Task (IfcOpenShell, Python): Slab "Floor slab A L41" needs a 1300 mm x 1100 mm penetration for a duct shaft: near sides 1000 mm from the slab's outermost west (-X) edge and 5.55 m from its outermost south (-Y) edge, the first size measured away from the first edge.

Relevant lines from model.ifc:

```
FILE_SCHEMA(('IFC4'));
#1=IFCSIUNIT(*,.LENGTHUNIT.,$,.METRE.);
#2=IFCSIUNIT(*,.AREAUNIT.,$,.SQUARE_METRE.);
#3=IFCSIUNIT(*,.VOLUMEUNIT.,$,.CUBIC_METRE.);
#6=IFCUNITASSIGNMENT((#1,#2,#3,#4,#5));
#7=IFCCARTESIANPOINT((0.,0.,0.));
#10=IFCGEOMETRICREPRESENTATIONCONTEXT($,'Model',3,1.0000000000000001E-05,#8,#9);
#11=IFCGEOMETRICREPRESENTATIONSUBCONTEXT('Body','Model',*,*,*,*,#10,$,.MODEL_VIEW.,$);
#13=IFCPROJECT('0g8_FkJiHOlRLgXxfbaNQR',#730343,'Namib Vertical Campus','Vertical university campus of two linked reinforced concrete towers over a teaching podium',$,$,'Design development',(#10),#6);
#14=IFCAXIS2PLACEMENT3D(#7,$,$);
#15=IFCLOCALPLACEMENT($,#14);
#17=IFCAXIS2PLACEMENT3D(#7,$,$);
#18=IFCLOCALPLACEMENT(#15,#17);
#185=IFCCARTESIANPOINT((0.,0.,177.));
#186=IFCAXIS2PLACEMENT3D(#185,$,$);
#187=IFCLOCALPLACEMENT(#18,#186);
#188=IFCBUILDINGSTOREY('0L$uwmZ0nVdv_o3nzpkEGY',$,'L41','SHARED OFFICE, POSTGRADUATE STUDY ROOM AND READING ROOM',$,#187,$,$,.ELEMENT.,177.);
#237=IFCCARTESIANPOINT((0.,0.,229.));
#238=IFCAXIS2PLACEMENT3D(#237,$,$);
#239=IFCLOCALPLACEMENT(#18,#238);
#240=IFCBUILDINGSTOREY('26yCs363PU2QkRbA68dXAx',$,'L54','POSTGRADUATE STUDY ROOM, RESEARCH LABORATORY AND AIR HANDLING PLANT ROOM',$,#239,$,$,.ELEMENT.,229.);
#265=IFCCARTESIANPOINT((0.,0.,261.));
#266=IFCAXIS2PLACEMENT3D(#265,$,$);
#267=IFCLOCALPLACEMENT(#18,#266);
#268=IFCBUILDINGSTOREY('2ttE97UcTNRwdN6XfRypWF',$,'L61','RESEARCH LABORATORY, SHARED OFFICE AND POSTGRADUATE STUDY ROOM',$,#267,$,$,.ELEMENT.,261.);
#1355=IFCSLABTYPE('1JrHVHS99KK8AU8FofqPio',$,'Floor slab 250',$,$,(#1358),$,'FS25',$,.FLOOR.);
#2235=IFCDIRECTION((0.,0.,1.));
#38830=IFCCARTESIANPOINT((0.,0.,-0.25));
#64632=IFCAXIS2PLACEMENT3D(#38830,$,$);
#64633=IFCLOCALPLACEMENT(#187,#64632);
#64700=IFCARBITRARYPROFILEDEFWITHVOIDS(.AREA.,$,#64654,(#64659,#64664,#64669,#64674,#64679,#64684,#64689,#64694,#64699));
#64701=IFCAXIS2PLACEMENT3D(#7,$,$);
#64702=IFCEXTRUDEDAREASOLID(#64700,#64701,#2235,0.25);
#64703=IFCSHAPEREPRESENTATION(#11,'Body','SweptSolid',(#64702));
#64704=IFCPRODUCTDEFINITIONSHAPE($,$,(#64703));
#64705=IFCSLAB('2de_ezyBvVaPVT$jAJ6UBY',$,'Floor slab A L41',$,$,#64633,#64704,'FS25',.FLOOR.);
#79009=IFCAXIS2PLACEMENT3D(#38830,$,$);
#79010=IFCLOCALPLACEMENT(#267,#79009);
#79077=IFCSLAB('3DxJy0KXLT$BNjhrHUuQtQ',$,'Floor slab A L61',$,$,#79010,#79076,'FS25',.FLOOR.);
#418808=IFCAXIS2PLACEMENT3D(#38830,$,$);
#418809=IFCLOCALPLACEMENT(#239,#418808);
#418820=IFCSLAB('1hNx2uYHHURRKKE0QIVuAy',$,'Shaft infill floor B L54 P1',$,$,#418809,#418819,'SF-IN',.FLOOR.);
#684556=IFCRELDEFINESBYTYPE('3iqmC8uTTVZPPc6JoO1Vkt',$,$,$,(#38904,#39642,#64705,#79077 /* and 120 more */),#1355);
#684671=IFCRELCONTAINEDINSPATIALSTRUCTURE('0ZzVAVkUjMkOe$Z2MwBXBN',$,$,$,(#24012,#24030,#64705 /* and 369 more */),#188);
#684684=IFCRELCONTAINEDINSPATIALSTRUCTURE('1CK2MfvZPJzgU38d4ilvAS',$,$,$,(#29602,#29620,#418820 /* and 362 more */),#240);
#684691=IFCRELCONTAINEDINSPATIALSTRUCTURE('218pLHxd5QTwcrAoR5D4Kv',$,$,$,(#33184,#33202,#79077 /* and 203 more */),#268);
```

```python
import numpy as np
import ifcopenshell
import ifcopenshell.api.feature
import ifcopenshell.api.geometry
import ifcopenshell.api.root
import ifcopenshell.geom
import ifcopenshell.util.placement
import ifcopenshell.util.representation
import ifcopenshell.util.shape
import ifcopenshell.util.unit

model = ifcopenshell.open("model.ifc")
unit_scale = ifcopenshell.util.unit.calculate_unit_scale(model)
settings = ifcopenshell.geom.settings()


def volume(element):
    """Net volume in cubic metres, openings subtracted."""
    shape = ifcopenshell.geom.create_shape(settings, element)
    return ifcopenshell.util.shape.get_volume(shape.geometry)


slab = model.by_id(64705)
before = volume(slab)

# Extent in the slab's own axes, in metres. The edges named are its -X and -Y sides.
slab_shape = ifcopenshell.geom.create_shape(settings, slab)
vertices = ifcopenshell.util.shape.get_vertices(slab_shape.geometry)
x_min, y_min, bottom = vertices.min(axis=0)
top = vertices[:, 2].max()

opening = ifcopenshell.api.root.create_entity(model, ifc_class="IfcOpeningElement", name="Duct shaft opening", predefined_type="OPENING")
context = ifcopenshell.util.representation.get_context(model, "Model", "Body", "MODEL_VIEW")
width, depth = 1.3, 1.1
outline = [(0.0, 0.0), (width, 0.0), (width, depth), (0.0, depth), (0.0, 0.0)]
# Overshoot both faces by 50 mm so the cut is clean.
shape = ifcopenshell.api.geometry.add_slab_representation(
    model, context=context, depth=top - bottom + 0.1, polyline=outline
)
ifcopenshell.api.geometry.assign_representation(model, product=opening, representation=shape)

matrix = ifcopenshell.util.placement.get_local_placement(slab.ObjectPlacement)
matrix[:, 3] = matrix @ np.append(np.array([x_min + 1, y_min + 5.55, bottom - 0.05]) / unit_scale, 1.0)
ifcopenshell.api.geometry.edit_object_placement(model, product=opening, matrix=matrix, is_si=False)
ifcopenshell.api.feature.add_feature(model, feature=opening, element=slab)

after = volume(slab)

print(f"slab volume {before:.3f} -> {after:.3f} m3")

model.write("model_edited.ifc")
```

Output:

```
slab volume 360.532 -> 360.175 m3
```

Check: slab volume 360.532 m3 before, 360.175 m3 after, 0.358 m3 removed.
